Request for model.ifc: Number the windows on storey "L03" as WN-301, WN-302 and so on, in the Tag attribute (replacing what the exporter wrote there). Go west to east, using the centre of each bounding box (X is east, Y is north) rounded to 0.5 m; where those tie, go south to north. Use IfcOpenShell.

First a look at what the model holds.

```python
import ifcopenshell
import ifcopenshell.util.element
import ifcopenshell.util.placement

model = ifcopenshell.open("model.ifc")
print(model.schema)
storey = next(s for s in model.by_type("IfcBuildingStorey") if s.Name == "L03")
windows = [e for e in ifcopenshell.util.element.get_decomposition(storey) if e.is_a("IfcWindow")]
for e in sorted(windows, key=lambda e: e.id()):
    origin = ifcopenshell.util.placement.get_local_placement(e.ObjectPlacement)[:3, 3]
    print(e.id(), e.Tag, e.Name, origin.round(2) + 0.0, sep=" | ")
```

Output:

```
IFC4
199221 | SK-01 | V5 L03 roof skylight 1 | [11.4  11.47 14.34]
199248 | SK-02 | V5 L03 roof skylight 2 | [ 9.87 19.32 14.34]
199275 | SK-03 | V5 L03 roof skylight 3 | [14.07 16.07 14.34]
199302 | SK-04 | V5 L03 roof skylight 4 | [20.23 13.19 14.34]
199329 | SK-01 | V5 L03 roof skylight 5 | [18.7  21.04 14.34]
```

```python
import ifcopenshell
import ifcopenshell.geom
import ifcopenshell.util.element
import ifcopenshell.util.shape

model = ifcopenshell.open("model.ifc")
settings = ifcopenshell.geom.settings()
settings.set("use-world-coords", True)


def centre(element):
    shape = ifcopenshell.geom.create_shape(settings, element)
    return ifcopenshell.util.shape.get_bbox_centroid(shape.geometry)


storey = next(s for s in model.by_type("IfcBuildingStorey") if s.Name == "L03")
windows = [e for e in ifcopenshell.util.element.get_decomposition(storey) if e.is_a("IfcWindow")]

# Insertion points can sit at a corner or the storey origin, so sort by the geometry (in metres).
centres = {e: centre(e) for e in windows}
windows.sort(key=lambda e: (round(centres[e][0] / 0.5), centres[e][1]))

for i, e in enumerate(windows, start=1):
    number = f"WN-3{i:02d}"
    e.Tag = number
    print(e.id(), number)

model.write("model-out.ifc")
```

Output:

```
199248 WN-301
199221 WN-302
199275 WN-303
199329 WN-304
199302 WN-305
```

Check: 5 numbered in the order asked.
